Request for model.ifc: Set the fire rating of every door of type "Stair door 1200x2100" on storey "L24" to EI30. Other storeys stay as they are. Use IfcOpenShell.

First a look at what the model holds.

```python
import ifcopenshell
import ifcopenshell.util.element

model = ifcopenshell.open("model.ifc")
print(model.schema)
storey = next(s for s in model.by_type("IfcBuildingStorey") if s.Name == "L24")
doors = [e for e in ifcopenshell.util.element.get_decomposition(storey) if e.is_a("IfcDoor")]
seen = {}
for e in doors:
    element_type = ifcopenshell.util.element.get_type(e)
    key = (element_type.Name if element_type != e and element_type else None, ifcopenshell.util.element.get_pset(e, "Pset_DoorCommon", "FireRating"))
    seen[key] = seen.get(key, 0) + 1
for (name, value), count in sorted(seen.items(), key=str):
    print(count, "x", name, "|", value)
```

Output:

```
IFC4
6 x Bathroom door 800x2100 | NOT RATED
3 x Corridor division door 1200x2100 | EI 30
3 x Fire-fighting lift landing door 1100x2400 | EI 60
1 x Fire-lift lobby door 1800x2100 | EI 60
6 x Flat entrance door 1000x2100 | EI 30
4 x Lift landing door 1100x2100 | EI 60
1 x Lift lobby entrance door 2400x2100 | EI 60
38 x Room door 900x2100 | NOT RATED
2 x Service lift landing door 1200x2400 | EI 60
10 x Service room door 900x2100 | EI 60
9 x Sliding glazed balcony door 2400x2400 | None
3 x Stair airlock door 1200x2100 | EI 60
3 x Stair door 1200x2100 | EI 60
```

```python
import ifcopenshell
import ifcopenshell.api.pset
import ifcopenshell.util.element

model = ifcopenshell.open("model.ifc")

storey = next(s for s in model.by_type("IfcBuildingStorey") if s.Name == "L24")
doors = [e for e in ifcopenshell.util.element.get_decomposition(storey) if e.is_a("IfcDoor")]

count = 0
for e in doors:
    element_type = ifcopenshell.util.element.get_type(e)
    if element_type in (None, e) or element_type.Name != "Stair door 1200x2100":
        continue
    # add_pset returns the element's existing set when there is one.
    pset = ifcopenshell.api.pset.add_pset(model, product=e, name="Pset_DoorCommon")
    ifcopenshell.api.pset.edit_pset(model, pset=pset, properties={"FireRating": "EI30"})
    count += 1

print(count, "doors updated")

model.write("model_rev.ifc")
```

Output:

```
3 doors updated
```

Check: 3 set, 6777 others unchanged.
